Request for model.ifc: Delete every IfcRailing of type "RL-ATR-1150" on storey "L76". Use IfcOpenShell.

First a look at what the model holds.

```python
import ifcopenshell
import ifcopenshell.util.element

model = ifcopenshell.open("model.ifc")
print(model.schema)
storey = next(s for s in model.by_type("IfcBuildingStorey") if s.Name == "L76")
railings = [e for e in ifcopenshell.util.element.get_decomposition(storey) if e.is_a("IfcRailing")]
seen = {}
for e in railings:
    element_type = ifcopenshell.util.element.get_type(e)
    name = element_type.Name if element_type not in (None, e) else None
    seen[name] = seen.get(name, 0) + 1
for name, count in sorted(seen.items(), key=str):
    print(count, "x", name)
```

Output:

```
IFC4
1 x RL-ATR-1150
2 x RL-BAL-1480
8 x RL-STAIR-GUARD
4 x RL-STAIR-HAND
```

```python
import ifcopenshell
import ifcopenshell.api.root
import ifcopenshell.util.element

model = ifcopenshell.open("model.ifc")

storey = next(s for s in model.by_type("IfcBuildingStorey") if s.Name == "L76")
railings = [e for e in ifcopenshell.util.element.get_decomposition(storey) if e.is_a("IfcRailing")]
targets = [e for e in railings if (t := ifcopenshell.util.element.get_type(e)) not in (None, e) and t.Name == "RL-ATR-1150"]

for e in targets:
    ifcopenshell.api.root.remove_product(model, product=e)
print(len(targets), "removed")

model.write("model-out.ifc")
```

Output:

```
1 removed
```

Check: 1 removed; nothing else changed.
